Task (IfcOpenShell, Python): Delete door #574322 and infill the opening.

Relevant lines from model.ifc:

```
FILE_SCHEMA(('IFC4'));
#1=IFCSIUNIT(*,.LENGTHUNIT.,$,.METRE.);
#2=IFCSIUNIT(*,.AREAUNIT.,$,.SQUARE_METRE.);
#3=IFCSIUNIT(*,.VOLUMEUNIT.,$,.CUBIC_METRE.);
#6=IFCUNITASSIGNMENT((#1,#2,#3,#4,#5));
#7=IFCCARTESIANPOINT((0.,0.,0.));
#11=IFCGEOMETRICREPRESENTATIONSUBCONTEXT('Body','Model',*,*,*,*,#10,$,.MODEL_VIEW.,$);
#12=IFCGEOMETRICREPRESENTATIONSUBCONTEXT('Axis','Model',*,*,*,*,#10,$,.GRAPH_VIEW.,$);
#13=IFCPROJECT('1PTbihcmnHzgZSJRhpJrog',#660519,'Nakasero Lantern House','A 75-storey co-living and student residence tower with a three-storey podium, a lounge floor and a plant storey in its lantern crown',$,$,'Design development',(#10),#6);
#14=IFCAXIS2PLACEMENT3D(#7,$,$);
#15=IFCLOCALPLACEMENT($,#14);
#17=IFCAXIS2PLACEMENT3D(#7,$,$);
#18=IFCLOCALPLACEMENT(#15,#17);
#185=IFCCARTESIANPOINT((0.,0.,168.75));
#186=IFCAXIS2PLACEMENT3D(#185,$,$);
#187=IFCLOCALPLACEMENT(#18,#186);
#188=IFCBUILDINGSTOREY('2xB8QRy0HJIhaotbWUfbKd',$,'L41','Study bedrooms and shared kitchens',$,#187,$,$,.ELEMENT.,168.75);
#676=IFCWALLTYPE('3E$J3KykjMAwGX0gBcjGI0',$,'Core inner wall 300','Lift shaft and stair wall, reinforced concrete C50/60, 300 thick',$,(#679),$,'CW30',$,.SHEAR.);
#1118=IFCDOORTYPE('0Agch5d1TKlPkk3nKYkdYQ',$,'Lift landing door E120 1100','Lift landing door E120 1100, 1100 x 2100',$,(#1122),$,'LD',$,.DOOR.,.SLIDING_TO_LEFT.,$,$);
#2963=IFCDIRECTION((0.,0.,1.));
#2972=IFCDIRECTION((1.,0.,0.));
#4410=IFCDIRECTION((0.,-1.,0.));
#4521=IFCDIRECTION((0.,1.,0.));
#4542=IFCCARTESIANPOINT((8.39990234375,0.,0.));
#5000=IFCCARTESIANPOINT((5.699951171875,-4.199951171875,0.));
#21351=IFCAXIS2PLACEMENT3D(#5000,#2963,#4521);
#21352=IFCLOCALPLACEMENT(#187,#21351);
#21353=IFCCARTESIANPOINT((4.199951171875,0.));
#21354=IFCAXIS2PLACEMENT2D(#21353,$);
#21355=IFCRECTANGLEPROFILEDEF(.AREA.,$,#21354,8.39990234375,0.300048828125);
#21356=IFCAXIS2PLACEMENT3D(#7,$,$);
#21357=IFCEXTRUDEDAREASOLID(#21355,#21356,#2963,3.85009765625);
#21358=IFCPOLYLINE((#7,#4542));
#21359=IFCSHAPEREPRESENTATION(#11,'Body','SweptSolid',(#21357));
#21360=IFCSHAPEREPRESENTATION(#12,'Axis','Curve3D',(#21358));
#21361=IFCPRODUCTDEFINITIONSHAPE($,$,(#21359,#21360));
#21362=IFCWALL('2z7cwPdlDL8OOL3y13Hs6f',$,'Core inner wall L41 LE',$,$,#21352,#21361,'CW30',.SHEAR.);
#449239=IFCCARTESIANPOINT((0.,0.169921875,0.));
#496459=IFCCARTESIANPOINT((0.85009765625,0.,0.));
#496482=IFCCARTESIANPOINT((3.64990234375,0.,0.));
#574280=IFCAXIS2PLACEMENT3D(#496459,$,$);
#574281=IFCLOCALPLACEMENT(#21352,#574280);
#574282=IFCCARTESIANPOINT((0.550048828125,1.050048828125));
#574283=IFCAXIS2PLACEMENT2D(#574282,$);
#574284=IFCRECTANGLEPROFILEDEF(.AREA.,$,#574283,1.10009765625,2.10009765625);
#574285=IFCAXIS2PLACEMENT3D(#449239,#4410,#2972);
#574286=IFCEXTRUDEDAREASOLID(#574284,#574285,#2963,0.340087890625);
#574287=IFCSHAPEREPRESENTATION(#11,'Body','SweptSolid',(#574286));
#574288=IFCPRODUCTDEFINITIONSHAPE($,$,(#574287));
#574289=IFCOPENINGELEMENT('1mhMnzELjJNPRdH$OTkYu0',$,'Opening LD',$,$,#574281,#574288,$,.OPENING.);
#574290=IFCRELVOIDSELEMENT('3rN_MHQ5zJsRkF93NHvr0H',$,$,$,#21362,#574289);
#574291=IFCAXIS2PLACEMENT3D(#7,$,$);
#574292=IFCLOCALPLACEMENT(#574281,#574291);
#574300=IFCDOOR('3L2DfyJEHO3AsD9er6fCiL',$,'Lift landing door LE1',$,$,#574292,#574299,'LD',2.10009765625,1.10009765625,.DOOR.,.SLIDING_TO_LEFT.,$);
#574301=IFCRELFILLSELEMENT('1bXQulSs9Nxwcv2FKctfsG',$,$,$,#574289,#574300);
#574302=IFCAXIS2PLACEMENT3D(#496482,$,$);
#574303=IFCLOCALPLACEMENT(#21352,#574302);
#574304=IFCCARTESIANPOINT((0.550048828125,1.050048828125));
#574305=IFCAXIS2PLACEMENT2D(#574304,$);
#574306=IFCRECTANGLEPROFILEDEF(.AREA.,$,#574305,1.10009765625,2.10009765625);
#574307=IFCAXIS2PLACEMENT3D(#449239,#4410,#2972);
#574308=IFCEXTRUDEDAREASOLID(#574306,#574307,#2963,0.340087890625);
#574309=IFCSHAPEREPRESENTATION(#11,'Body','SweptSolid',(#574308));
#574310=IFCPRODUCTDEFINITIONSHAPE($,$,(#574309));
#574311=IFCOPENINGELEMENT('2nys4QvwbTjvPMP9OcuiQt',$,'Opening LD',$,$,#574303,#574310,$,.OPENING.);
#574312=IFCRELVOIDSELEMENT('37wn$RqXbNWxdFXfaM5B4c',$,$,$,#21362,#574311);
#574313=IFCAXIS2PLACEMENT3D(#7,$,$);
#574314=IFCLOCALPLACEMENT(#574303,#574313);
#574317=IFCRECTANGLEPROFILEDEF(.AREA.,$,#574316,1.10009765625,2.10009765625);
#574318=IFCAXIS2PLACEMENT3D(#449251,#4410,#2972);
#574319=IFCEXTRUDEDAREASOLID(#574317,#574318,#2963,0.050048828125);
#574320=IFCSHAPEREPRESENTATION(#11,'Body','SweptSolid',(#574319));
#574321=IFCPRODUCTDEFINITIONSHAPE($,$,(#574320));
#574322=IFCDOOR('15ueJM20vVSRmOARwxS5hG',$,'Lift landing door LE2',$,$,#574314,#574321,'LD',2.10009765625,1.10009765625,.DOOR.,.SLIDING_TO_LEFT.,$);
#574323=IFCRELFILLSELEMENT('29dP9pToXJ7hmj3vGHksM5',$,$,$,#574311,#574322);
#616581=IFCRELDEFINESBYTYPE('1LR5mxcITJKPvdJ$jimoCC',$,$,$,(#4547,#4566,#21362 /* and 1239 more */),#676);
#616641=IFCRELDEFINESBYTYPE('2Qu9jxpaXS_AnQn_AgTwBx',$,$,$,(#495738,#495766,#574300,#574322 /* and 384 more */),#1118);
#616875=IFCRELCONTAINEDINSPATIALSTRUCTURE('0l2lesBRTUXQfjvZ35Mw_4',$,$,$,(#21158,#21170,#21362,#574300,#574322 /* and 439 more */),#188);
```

```python
import ifcopenshell
import ifcopenshell.api.feature
import ifcopenshell.api.root
import ifcopenshell.geom
import ifcopenshell.util.shape

model = ifcopenshell.open("model.ifc")
settings = ifcopenshell.geom.settings()


def volume(element):
    """Net volume in cubic metres, openings subtracted."""
    shape = ifcopenshell.geom.create_shape(settings, element)
    return ifcopenshell.util.shape.get_volume(shape.geometry)


door = model.by_guid("15ueJM20vVSRmOARwxS5hG")
opening = door.FillsVoids[0].RelatingOpeningElement
wall = opening.VoidsElements[0].RelatingBuildingElement
before = volume(wall)

ifcopenshell.api.root.remove_product(model, product=door)
ifcopenshell.api.feature.remove_feature(model, feature=opening)

after = volume(wall)

print(f"wall volume {before:.3f} -> {after:.3f} m3")

model.write("model_rev.ifc")
```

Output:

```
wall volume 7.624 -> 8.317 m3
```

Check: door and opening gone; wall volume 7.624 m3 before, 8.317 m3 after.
